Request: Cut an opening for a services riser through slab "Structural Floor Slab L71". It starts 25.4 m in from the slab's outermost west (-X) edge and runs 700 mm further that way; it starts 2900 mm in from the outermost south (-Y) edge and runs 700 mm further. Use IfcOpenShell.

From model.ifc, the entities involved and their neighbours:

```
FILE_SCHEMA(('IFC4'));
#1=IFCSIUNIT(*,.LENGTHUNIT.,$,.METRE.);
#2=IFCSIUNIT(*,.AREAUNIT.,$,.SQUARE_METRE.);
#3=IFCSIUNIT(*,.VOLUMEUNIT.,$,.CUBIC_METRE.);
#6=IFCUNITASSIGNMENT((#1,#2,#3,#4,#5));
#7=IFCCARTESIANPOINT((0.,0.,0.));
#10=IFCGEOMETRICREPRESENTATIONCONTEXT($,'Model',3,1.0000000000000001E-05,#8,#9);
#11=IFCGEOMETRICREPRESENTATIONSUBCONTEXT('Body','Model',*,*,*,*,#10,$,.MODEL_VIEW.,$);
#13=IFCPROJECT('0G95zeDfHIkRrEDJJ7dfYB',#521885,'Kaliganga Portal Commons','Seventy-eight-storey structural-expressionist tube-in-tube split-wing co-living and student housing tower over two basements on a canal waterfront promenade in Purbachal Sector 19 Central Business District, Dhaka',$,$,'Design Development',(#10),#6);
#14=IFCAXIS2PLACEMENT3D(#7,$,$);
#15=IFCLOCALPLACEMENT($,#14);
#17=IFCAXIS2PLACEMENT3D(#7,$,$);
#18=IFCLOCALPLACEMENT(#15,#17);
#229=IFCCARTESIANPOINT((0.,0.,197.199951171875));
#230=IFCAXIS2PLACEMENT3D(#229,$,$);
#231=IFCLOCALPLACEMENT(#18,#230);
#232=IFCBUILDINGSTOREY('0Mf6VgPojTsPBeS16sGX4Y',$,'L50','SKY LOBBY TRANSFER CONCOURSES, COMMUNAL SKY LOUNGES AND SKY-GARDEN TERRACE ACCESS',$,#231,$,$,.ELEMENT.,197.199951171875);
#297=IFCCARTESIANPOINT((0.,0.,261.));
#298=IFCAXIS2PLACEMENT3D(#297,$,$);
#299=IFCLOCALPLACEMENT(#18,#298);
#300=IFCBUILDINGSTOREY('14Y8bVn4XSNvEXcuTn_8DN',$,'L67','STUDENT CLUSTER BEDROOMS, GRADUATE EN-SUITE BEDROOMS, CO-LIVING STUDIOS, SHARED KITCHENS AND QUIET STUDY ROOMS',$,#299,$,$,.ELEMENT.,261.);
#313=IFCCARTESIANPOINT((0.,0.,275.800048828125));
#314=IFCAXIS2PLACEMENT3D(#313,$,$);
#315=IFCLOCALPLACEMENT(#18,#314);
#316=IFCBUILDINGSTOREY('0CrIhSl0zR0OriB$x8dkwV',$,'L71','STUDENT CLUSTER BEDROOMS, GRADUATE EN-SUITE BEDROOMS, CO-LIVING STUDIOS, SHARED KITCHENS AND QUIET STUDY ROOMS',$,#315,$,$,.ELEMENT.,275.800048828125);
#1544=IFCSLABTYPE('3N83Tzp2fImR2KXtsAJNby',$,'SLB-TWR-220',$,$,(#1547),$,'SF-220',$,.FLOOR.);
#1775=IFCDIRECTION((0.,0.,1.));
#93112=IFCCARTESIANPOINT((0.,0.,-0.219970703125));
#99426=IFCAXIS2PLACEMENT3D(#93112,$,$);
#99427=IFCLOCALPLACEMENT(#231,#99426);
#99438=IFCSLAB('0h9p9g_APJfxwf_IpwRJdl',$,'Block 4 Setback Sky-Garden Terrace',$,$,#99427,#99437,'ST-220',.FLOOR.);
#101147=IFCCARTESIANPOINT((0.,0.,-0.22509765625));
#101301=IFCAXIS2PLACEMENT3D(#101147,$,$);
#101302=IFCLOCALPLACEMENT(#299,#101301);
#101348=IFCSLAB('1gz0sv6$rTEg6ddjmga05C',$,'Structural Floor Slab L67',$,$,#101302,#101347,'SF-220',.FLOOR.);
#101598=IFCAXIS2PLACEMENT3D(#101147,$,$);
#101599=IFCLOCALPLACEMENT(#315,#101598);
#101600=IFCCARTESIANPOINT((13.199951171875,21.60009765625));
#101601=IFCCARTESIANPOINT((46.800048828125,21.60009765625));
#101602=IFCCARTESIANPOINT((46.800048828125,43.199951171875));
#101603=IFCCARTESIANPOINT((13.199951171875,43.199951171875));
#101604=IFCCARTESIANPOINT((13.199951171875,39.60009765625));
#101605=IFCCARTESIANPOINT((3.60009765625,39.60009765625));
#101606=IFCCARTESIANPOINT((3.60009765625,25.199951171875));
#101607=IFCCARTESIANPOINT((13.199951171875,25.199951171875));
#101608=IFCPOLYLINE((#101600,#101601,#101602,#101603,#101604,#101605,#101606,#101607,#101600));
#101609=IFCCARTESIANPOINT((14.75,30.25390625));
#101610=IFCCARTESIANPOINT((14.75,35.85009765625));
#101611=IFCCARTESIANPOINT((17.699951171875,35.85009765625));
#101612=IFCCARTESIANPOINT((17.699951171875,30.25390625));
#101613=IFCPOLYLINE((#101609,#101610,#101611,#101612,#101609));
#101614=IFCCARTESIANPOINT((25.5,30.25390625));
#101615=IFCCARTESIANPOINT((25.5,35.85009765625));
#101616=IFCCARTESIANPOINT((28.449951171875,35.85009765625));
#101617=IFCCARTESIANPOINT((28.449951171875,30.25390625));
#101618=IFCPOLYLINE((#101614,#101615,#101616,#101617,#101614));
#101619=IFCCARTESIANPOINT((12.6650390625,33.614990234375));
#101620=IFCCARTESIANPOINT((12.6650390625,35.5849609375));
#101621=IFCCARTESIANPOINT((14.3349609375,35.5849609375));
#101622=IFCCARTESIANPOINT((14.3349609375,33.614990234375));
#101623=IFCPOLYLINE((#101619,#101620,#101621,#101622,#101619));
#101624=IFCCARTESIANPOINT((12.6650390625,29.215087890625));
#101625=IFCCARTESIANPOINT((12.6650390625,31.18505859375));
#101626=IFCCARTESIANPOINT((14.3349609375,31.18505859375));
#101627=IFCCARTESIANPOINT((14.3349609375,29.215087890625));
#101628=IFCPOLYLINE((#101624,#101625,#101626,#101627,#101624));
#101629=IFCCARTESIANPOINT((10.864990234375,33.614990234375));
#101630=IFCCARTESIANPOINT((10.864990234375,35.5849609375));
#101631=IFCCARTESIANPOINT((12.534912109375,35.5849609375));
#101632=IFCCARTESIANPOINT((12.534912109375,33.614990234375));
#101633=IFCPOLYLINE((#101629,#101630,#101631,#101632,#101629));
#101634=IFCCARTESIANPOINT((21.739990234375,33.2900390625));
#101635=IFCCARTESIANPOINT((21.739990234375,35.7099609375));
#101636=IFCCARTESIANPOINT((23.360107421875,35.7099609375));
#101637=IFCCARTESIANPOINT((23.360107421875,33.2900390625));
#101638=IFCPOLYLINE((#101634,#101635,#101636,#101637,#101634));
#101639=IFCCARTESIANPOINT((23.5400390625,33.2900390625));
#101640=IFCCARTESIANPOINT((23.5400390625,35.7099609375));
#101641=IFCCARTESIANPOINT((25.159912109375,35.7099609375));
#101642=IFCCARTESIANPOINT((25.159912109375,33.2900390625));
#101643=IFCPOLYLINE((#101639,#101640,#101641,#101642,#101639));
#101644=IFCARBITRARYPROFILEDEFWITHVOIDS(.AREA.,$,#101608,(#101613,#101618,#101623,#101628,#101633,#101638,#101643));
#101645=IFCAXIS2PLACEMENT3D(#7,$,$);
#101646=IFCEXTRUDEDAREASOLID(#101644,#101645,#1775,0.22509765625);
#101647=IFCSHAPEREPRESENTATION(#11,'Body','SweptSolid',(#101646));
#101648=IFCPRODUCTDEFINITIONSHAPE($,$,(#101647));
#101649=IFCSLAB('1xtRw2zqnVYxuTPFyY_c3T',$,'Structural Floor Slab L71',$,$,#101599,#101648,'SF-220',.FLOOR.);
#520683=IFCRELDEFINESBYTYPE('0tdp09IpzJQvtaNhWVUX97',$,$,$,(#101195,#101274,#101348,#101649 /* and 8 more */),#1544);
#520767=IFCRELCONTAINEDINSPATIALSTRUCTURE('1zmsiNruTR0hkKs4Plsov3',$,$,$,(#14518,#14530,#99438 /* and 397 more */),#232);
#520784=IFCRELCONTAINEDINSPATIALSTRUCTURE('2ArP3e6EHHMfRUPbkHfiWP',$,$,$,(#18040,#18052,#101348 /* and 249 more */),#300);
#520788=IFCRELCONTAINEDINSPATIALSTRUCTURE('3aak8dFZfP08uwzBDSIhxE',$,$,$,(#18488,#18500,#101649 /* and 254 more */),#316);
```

```python
import numpy as np
import ifcopenshell
import ifcopenshell.api.feature
import ifcopenshell.api.geometry
import ifcopenshell.api.root
import ifcopenshell.geom
import ifcopenshell.util.placement
import ifcopenshell.util.representation
import ifcopenshell.util.shape
import ifcopenshell.util.unit

model = ifcopenshell.open("model.ifc")
unit_scale = ifcopenshell.util.unit.calculate_unit_scale(model)
settings = ifcopenshell.geom.settings()


def volume(element):
    """Net volume in cubic metres, openings subtracted."""
    shape = ifcopenshell.geom.create_shape(settings, element)
    return ifcopenshell.util.shape.get_volume(shape.geometry)


slab = model.by_guid("1xtRw2zqnVYxuTPFyY_c3T")
before = volume(slab)

# Extent in the slab's own axes, in metres. The edges named are its -X and -Y sides.
slab_shape = ifcopenshell.geom.create_shape(settings, slab)
vertices = ifcopenshell.util.shape.get_vertices(slab_shape.geometry)
x_min, y_min, bottom = vertices.min(axis=0)
top = vertices[:, 2].max()

opening = ifcopenshell.api.root.create_entity(model, ifc_class="IfcOpeningElement", name="Services riser opening", predefined_type="OPENING")
context = ifcopenshell.util.representation.get_context(model, "Model", "Body", "MODEL_VIEW")
width, depth = 0.7, 0.7
outline = [(0.0, 0.0), (width, 0.0), (width, depth), (0.0, depth), (0.0, 0.0)]
# Overshoot both faces by 50 mm so the cut is clean.
shape = ifcopenshell.api.geometry.add_slab_representation(
    model, context=context, depth=top - bottom + 0.1, polyline=outline
)
ifcopenshell.api.geometry.assign_representation(model, product=opening, representation=shape)

matrix = ifcopenshell.util.placement.get_local_placement(slab.ObjectPlacement)
matrix[:, 3] = matrix @ np.append(np.array([x_min + 25.4, y_min + 2.9, bottom - 0.05]) / unit_scale, 1.0)
ifcopenshell.api.geometry.edit_object_placement(model, product=opening, matrix=matrix, is_si=False)
ifcopenshell.api.feature.add_feature(model, feature=opening, element=slab)

after = volume(slab)

print(f"slab volume {before:.3f} -> {after:.3f} m3")

model.write("model_v2.ifc")
```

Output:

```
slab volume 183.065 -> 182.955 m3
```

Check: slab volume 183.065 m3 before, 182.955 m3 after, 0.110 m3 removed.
